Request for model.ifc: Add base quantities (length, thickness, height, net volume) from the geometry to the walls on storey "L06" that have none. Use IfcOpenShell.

First a look at what the model holds.

```python
import ifcopenshell
import ifcopenshell.util.element
import ifcopenshell.util.unit

model = ifcopenshell.open("model.ifc")
print(model.schema)
for unit_type in ("LENGTHUNIT", "AREAUNIT", "VOLUMEUNIT"):
    print(unit_type, ifcopenshell.util.unit.calculate_unit_scale(model, unit_type))
storey = next(s for s in model.by_type("IfcBuildingStorey") if s.Name == "L06")
walls = [e for e in ifcopenshell.util.element.get_decomposition(storey) if e.is_a("IfcWall")]
for e in sorted(walls, key=lambda e: e.id()):
    print(e.id(), e.is_a(), e.Name, list(ifcopenshell.util.element.get_psets(e, qtos_only=True)), sep=" | ")
```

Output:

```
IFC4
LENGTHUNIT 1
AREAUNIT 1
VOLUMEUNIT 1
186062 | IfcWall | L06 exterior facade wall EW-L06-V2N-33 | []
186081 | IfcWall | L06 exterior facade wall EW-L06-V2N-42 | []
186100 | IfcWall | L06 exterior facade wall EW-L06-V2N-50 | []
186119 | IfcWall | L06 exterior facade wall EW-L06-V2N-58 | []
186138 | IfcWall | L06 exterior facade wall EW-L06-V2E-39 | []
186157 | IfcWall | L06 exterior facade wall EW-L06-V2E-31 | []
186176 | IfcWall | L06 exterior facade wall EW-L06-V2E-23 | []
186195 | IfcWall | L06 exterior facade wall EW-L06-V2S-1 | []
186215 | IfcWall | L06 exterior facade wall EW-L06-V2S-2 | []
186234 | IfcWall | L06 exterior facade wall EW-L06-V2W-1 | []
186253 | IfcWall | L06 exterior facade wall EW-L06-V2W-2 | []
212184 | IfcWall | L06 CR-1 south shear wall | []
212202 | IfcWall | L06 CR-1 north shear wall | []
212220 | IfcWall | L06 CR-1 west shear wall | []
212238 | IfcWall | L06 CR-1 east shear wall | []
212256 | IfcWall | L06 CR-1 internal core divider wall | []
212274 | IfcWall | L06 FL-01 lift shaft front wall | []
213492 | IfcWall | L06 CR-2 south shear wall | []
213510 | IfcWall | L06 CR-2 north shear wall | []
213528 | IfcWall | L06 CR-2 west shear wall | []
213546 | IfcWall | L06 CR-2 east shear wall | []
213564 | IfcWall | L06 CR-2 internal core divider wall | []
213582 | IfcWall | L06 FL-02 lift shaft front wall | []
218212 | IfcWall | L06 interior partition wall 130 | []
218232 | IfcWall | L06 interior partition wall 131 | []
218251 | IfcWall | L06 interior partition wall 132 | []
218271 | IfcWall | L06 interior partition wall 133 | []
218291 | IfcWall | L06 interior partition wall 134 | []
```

```python
import ifcopenshell
import ifcopenshell.api.pset
import ifcopenshell.geom
import ifcopenshell.util.element
import ifcopenshell.util.shape
import ifcopenshell.util.unit

model = ifcopenshell.open("model.ifc")
unit_scale = ifcopenshell.util.unit.calculate_unit_scale(model)
volume_scale = ifcopenshell.util.unit.calculate_unit_scale(model, "VOLUMEUNIT")
settings = ifcopenshell.geom.settings()

storey = next(s for s in model.by_type("IfcBuildingStorey") if s.Name == "L06")
walls = [e for e in ifcopenshell.util.element.get_decomposition(storey) if e.is_a("IfcWall")]

for e in sorted(walls, key=lambda e: e.id()):
    if ifcopenshell.util.element.get_psets(e, qtos_only=True, should_inherit=False):
        continue
    # Geometry comes back in metres, in the element's own axes.
    shape = ifcopenshell.geom.create_shape(settings, e)
    values = {
        "Length": ifcopenshell.util.shape.get_x(shape.geometry) / unit_scale,
        "Width": ifcopenshell.util.shape.get_y(shape.geometry) / unit_scale,
        "Height": ifcopenshell.util.shape.get_z(shape.geometry) / unit_scale,
        "NetVolume": ifcopenshell.util.shape.get_volume(shape.geometry) / volume_scale,
    }
    qto = ifcopenshell.api.pset.add_qto(model, product=e, name="Qto_WallBaseQuantities")
    ifcopenshell.api.pset.edit_qto(model, qto=qto, properties=values)
    print(e.id(), {k: round(v, 3) for k, v in values.items()})

model.write("model_edited.ifc")
```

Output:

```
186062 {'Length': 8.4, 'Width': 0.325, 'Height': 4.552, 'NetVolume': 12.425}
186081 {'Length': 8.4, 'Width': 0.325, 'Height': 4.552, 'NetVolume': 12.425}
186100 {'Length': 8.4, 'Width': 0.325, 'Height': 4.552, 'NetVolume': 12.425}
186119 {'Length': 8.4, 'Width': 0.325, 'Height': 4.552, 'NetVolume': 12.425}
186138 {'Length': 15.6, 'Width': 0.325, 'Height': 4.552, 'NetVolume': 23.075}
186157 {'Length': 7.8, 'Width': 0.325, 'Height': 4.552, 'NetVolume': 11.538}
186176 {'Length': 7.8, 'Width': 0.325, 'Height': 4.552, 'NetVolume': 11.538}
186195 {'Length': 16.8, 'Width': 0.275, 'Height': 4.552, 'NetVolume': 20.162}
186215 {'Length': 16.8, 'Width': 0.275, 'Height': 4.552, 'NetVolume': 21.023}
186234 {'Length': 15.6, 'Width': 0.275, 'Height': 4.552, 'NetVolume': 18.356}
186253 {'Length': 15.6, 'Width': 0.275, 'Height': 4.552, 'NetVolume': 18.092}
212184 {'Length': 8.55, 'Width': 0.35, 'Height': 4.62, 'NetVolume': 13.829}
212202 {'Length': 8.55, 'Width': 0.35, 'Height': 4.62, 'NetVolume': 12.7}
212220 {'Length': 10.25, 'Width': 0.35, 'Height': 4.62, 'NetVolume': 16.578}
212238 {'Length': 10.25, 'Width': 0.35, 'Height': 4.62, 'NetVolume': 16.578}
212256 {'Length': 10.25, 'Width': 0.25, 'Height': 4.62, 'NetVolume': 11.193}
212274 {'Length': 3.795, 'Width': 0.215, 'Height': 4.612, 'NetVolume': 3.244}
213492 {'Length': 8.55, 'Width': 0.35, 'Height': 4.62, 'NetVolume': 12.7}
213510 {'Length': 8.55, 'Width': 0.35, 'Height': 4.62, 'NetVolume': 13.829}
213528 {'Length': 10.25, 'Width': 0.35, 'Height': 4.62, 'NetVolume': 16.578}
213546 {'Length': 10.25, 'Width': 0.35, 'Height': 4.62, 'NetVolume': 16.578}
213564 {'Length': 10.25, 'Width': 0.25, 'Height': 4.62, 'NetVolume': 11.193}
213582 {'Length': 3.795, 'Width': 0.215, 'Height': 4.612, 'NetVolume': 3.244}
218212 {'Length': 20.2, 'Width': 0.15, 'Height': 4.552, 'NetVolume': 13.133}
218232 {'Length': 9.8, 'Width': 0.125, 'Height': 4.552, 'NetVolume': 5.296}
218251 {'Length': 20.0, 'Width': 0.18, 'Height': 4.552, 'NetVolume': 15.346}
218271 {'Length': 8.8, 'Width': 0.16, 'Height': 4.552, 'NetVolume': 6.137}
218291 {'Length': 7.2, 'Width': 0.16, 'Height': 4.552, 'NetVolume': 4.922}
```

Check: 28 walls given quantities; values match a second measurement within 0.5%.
